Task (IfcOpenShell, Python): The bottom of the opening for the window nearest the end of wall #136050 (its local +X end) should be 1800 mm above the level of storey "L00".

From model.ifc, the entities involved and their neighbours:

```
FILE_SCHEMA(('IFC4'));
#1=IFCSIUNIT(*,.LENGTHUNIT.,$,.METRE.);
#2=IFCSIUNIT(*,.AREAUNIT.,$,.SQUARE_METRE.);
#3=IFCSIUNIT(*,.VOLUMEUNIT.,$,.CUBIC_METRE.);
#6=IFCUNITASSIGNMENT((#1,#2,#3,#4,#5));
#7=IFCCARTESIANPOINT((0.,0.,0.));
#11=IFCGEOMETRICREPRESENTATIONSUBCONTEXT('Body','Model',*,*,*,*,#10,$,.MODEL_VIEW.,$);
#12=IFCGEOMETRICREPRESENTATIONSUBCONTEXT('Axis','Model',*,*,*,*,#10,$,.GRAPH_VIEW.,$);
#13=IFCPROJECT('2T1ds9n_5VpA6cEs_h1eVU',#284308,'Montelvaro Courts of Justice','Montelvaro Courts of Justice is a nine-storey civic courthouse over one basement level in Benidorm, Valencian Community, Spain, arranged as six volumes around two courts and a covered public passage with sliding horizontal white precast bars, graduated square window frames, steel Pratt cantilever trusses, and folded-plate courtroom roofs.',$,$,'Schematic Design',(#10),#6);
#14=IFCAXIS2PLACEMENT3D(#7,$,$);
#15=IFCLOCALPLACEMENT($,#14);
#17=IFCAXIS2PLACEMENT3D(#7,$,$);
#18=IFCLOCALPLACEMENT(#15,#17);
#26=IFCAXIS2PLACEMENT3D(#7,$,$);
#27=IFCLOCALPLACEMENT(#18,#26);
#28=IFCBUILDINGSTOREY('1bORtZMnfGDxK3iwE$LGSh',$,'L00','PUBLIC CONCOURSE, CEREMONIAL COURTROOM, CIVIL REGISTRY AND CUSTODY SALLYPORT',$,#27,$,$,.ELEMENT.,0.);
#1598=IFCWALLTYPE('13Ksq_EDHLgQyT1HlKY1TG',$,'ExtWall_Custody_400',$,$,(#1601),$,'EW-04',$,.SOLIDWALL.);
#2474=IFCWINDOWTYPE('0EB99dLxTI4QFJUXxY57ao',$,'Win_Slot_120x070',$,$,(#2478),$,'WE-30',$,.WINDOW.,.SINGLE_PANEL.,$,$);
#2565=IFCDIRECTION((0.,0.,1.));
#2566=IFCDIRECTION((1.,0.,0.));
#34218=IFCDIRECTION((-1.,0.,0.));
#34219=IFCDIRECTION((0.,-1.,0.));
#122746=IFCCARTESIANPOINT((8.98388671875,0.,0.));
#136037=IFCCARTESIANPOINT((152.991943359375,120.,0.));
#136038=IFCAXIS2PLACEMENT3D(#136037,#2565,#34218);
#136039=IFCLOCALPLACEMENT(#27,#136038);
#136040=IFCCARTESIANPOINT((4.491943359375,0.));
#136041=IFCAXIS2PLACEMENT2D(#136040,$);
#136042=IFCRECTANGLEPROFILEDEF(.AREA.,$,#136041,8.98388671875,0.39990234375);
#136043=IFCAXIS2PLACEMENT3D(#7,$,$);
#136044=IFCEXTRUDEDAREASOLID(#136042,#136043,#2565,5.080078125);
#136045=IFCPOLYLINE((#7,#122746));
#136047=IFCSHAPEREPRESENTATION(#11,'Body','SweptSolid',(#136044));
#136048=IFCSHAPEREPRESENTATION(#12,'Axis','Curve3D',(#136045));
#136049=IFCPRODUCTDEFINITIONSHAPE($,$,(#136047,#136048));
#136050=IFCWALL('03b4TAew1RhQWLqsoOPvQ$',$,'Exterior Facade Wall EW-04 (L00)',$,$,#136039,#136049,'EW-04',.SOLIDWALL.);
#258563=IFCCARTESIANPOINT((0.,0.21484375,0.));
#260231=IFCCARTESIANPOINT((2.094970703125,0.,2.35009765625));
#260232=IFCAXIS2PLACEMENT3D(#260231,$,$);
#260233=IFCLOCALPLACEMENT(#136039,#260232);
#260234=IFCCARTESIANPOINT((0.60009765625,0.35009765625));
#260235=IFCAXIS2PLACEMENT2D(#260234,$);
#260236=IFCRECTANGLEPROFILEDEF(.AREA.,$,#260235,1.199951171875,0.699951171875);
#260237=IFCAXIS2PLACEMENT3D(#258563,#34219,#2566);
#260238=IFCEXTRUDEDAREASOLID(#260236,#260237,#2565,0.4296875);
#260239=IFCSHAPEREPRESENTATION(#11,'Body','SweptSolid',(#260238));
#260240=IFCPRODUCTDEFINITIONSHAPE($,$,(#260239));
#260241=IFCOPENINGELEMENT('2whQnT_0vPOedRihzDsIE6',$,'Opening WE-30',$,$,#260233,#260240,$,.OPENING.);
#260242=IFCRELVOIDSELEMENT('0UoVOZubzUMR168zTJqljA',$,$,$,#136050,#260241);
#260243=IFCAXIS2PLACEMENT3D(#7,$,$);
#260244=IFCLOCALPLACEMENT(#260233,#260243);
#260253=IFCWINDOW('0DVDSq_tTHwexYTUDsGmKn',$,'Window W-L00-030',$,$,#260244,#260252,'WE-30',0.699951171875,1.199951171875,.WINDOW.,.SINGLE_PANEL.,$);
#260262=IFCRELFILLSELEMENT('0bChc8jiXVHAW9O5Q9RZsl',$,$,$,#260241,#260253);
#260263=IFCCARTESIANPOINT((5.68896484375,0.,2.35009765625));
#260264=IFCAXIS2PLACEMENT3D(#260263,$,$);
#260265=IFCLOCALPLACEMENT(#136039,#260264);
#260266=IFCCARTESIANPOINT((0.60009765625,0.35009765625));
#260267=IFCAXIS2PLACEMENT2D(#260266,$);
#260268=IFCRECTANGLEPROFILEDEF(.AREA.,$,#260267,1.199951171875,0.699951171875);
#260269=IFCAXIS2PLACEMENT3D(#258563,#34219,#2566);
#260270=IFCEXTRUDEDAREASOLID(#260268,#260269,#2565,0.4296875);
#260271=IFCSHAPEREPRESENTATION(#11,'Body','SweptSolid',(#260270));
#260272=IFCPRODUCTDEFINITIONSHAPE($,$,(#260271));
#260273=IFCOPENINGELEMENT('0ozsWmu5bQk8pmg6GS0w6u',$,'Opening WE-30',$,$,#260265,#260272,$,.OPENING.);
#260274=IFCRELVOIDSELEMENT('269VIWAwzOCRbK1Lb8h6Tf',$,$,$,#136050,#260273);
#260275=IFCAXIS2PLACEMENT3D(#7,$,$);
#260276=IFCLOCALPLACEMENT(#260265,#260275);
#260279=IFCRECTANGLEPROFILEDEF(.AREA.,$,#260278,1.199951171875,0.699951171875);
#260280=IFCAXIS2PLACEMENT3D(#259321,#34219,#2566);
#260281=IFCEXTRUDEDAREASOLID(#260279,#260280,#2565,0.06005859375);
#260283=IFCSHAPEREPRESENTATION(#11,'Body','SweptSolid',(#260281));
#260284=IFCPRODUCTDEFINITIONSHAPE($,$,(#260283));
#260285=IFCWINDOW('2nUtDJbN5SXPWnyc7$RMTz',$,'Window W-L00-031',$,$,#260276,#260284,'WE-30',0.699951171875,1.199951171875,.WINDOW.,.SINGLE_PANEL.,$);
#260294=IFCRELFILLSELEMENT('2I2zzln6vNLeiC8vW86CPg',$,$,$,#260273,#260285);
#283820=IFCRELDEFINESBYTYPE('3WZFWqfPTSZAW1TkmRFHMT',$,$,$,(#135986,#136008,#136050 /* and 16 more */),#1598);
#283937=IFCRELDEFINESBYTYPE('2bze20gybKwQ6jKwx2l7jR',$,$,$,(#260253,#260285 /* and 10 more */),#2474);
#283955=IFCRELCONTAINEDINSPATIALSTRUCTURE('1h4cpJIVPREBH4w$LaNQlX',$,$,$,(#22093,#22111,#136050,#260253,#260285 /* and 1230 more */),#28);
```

```python
import numpy as np
import ifcopenshell
import ifcopenshell.api.geometry
import ifcopenshell.geom
import ifcopenshell.util.element
import ifcopenshell.util.placement
import ifcopenshell.util.shape
import ifcopenshell.util.unit

model = ifcopenshell.open("model.ifc")
unit_scale = ifcopenshell.util.unit.calculate_unit_scale(model)

window = model.by_guid("2nUtDJbN5SXPWnyc7$RMTz")
opening = window.FillsVoids[0].RelatingOpeningElement
storey = ifcopenshell.util.element.get_container(window, ifc_class="IfcBuildingStorey")
level = ifcopenshell.util.placement.get_local_placement(storey.ObjectPlacement)[2, 3]

# The opening's origin need not be at the sill, so measure its lowest point.
shape = ifcopenshell.geom.create_shape(ifcopenshell.geom.settings(), opening)
bottom = ifcopenshell.util.shape.get_shape_bottom_elevation(shape, shape.geometry) / unit_scale
dz = level + 1.8 / unit_scale - bottom

shift = np.array([0.0, 0.0, dz])
# The window is placed relative to its opening, so it follows when the opening moves.
matrix = ifcopenshell.util.placement.get_local_placement(opening.ObjectPlacement)
matrix[:3, 3] += shift
ifcopenshell.api.geometry.edit_object_placement(
    model, product=opening, matrix=matrix, is_si=False, should_transform_children=True
)

print(f"moved by {dz * unit_scale:+.3f} m")

model.write("model-out.ifc")
```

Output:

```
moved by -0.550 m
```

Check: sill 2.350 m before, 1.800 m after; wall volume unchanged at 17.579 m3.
